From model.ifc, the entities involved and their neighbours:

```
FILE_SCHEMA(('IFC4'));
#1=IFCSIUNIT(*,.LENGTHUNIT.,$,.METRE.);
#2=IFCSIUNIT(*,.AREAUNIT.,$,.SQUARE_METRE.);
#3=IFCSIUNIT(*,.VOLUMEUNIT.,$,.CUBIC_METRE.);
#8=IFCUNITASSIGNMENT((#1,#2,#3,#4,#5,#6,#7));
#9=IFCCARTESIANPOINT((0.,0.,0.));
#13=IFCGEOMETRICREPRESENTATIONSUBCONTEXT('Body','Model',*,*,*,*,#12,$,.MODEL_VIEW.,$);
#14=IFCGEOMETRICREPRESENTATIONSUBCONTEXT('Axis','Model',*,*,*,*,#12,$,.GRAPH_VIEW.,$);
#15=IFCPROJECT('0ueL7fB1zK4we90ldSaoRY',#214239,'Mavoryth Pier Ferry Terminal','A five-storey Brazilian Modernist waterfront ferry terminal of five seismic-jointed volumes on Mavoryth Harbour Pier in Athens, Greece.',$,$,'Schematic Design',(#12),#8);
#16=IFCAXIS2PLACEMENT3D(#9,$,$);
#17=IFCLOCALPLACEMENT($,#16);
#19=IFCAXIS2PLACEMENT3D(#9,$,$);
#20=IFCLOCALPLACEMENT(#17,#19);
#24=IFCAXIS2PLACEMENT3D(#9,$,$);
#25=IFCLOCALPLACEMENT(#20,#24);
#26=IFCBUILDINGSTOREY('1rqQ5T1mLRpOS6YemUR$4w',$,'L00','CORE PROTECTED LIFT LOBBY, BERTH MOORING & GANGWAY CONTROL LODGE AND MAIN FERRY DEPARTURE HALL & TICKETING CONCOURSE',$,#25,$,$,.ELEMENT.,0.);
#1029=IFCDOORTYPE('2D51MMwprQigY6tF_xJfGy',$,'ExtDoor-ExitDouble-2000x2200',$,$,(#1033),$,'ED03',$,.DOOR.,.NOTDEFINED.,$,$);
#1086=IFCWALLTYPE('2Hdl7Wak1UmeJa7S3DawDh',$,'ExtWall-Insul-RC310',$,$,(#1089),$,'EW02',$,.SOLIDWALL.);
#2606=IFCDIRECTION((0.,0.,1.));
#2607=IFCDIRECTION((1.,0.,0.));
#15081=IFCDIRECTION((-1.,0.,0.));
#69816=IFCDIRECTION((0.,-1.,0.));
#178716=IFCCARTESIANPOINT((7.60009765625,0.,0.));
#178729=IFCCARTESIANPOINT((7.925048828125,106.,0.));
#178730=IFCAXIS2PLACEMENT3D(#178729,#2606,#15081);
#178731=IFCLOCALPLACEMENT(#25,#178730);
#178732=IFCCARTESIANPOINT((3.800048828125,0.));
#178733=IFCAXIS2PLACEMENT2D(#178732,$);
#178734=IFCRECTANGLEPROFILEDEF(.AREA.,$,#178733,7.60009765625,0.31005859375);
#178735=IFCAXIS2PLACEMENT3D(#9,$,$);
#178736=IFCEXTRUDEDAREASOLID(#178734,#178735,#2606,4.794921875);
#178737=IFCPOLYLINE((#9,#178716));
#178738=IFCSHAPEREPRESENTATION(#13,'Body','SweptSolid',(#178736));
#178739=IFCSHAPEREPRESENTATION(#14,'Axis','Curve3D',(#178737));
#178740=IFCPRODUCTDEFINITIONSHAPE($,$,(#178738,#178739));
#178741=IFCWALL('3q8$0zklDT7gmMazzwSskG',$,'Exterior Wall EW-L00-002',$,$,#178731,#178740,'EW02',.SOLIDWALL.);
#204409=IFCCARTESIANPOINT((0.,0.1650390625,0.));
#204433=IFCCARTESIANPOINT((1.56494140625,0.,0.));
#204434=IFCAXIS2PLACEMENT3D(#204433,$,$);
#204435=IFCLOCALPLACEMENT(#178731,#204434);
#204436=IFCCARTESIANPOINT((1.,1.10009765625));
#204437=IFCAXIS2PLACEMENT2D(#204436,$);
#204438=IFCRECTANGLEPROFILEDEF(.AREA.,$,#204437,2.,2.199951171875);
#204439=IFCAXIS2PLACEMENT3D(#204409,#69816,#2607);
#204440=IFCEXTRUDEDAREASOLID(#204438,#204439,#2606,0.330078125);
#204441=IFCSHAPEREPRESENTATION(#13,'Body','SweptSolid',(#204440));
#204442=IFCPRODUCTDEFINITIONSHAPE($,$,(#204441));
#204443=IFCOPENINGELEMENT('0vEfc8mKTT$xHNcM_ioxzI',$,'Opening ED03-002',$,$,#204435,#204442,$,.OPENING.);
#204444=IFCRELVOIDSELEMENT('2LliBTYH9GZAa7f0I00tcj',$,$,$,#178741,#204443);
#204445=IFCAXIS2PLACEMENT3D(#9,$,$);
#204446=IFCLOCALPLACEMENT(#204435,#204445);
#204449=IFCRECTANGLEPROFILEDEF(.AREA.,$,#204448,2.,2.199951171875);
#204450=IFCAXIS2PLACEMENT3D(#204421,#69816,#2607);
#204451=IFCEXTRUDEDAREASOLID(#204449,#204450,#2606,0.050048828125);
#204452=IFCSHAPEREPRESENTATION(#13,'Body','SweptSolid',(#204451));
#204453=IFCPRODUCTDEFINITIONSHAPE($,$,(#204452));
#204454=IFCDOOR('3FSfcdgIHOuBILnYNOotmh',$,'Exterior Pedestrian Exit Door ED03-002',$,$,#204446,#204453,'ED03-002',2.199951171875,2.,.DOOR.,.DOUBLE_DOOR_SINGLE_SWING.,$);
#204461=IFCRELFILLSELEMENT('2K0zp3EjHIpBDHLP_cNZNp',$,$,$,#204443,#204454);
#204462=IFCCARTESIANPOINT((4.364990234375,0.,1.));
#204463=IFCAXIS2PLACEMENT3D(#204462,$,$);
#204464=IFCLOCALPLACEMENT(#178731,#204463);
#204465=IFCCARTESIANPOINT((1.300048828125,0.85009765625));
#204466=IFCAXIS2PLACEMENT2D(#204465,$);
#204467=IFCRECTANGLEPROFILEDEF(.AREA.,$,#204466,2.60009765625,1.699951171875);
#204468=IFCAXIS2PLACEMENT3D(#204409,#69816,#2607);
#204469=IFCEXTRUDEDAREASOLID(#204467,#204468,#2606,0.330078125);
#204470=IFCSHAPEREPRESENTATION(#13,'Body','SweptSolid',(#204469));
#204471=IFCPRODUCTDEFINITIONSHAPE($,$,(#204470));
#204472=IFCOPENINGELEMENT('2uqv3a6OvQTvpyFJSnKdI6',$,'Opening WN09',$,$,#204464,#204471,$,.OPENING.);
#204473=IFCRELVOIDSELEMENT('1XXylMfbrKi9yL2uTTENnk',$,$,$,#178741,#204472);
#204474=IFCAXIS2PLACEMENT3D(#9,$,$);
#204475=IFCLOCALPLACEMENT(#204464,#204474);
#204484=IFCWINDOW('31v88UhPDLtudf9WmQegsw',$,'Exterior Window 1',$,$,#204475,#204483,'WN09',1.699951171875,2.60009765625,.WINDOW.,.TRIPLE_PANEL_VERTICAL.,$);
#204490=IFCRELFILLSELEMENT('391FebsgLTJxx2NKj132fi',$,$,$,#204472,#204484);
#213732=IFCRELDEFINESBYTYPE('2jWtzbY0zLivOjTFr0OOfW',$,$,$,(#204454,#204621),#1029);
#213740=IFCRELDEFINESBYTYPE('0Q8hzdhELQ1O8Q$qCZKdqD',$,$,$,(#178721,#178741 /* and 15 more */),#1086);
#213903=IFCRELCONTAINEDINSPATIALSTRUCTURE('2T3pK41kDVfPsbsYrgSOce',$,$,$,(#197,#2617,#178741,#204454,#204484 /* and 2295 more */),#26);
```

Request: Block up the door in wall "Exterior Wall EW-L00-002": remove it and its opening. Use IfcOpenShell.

```python
import ifcopenshell
import ifcopenshell.api.feature
import ifcopenshell.api.root
import ifcopenshell.geom
import ifcopenshell.util.shape

model = ifcopenshell.open("model.ifc")
settings = ifcopenshell.geom.settings()


def volume(element):
    """Net volume in cubic metres, openings subtracted."""
    shape = ifcopenshell.geom.create_shape(settings, element)
    return ifcopenshell.util.shape.get_volume(shape.geometry)


door = model.by_guid("3FSfcdgIHOuBILnYNOotmh")
opening = door.FillsVoids[0].RelatingOpeningElement
wall = opening.VoidsElements[0].RelatingBuildingElement
before = volume(wall)

ifcopenshell.api.root.remove_product(model, product=door)
ifcopenshell.api.feature.remove_feature(model, feature=opening)

after = volume(wall)

print(f"wall volume {before:.3f} -> {after:.3f} m3")

model.write("model_updated.ifc")
```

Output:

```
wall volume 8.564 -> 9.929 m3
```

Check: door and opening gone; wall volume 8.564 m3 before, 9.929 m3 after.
